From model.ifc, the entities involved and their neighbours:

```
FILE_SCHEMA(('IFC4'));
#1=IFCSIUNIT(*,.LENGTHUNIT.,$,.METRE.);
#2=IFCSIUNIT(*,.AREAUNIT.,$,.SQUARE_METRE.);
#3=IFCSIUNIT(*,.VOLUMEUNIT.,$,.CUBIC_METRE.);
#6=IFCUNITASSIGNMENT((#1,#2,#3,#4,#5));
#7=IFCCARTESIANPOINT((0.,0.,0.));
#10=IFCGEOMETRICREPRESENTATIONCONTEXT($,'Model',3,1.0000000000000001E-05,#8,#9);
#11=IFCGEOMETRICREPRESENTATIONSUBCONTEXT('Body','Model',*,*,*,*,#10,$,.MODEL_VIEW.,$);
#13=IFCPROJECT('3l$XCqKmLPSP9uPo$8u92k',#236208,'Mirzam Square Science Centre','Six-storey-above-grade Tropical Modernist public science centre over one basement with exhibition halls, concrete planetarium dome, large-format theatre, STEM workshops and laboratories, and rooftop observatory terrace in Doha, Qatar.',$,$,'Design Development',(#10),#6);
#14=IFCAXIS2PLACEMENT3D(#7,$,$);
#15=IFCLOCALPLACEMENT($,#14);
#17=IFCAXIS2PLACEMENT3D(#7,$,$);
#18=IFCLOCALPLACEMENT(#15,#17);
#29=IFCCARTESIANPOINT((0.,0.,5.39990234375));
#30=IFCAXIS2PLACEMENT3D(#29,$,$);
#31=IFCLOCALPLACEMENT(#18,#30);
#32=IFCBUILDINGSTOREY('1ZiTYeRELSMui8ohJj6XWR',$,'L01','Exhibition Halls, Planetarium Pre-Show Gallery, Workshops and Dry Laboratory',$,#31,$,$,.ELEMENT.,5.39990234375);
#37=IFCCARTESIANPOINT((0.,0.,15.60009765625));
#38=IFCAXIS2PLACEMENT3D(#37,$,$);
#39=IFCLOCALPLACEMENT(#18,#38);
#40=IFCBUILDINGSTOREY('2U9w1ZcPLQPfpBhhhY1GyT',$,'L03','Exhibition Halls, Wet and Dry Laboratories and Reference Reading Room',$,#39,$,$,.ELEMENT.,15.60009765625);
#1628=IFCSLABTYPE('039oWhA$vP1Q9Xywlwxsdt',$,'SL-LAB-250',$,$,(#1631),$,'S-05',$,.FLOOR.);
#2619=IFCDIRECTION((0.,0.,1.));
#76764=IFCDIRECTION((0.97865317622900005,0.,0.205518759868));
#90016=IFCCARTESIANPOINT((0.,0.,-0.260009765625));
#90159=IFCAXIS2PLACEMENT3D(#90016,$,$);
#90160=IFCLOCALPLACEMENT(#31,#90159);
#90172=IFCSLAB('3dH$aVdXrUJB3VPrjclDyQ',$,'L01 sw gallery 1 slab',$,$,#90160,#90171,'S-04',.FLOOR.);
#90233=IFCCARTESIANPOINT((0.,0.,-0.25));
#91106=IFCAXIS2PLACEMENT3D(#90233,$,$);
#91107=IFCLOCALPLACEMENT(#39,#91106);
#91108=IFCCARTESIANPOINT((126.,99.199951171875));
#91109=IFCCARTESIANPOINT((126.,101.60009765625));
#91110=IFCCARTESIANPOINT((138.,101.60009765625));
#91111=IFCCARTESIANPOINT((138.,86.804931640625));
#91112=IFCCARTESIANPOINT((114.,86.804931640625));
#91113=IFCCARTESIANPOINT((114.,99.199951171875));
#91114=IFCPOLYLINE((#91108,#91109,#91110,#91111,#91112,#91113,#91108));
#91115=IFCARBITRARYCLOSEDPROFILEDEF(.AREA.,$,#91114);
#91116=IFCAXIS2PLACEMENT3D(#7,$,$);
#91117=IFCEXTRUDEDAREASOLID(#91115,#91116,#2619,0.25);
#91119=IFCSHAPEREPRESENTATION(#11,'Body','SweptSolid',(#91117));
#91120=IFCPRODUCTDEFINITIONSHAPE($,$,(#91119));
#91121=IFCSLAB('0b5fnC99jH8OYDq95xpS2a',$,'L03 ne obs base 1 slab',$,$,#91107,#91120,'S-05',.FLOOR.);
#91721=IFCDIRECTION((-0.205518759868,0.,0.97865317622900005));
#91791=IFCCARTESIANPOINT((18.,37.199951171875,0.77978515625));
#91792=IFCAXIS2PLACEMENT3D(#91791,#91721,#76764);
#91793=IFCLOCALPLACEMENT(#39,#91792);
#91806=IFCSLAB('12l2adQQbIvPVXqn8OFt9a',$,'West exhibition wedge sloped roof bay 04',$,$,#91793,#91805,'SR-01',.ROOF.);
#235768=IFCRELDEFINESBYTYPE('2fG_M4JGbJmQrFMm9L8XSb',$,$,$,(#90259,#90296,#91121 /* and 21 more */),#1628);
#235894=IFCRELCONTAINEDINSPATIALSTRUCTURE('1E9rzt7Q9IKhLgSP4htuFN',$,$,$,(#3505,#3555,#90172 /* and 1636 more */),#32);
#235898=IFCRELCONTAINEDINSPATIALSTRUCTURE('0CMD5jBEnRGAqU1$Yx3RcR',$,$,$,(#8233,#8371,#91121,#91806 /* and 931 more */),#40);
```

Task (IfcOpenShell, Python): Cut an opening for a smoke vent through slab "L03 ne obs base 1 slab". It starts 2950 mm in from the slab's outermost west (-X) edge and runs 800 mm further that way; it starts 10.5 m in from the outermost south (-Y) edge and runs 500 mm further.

```python
import numpy as np
import ifcopenshell
import ifcopenshell.api.feature
import ifcopenshell.api.geometry
import ifcopenshell.api.root
import ifcopenshell.geom
import ifcopenshell.util.placement
import ifcopenshell.util.representation
import ifcopenshell.util.shape
import ifcopenshell.util.unit

model = ifcopenshell.open("model.ifc")
unit_scale = ifcopenshell.util.unit.calculate_unit_scale(model)
settings = ifcopenshell.geom.settings()


def volume(element):
    """Net volume in cubic metres, openings subtracted."""
    shape = ifcopenshell.geom.create_shape(settings, element)
    return ifcopenshell.util.shape.get_volume(shape.geometry)


slab = model.by_guid("0b5fnC99jH8OYDq95xpS2a")
before = volume(slab)

# Extent in the slab's own axes, in metres. The edges named are its -X and -Y sides.
slab_shape = ifcopenshell.geom.create_shape(settings, slab)
vertices = ifcopenshell.util.shape.get_vertices(slab_shape.geometry)
x_min, y_min, bottom = vertices.min(axis=0)
top = vertices[:, 2].max()

opening = ifcopenshell.api.root.create_entity(model, ifc_class="IfcOpeningElement", name="Smoke vent opening", predefined_type="OPENING")
context = ifcopenshell.util.representation.get_context(model, "Model", "Body", "MODEL_VIEW")
width, depth = 0.8, 0.5
outline = [(0.0, 0.0), (width, 0.0), (width, depth), (0.0, depth), (0.0, 0.0)]
# Overshoot both faces by 50 mm so the cut is clean.
shape = ifcopenshell.api.geometry.add_slab_representation(
    model, context=context, depth=top - bottom + 0.1, polyline=outline
)
ifcopenshell.api.geometry.assign_representation(model, product=opening, representation=shape)

matrix = ifcopenshell.util.placement.get_local_placement(slab.ObjectPlacement)
matrix[:, 3] = matrix @ np.append(np.array([x_min + 2.95, y_min + 10.5, bottom - 0.05]) / unit_scale, 1.0)
ifcopenshell.api.geometry.edit_object_placement(model, product=opening, matrix=matrix, is_si=False)
ifcopenshell.api.feature.add_feature(model, feature=opening, element=slab)

after = volume(slab)

print(f"slab volume {before:.3f} -> {after:.3f} m3")

model.write("model_rev.ifc")
```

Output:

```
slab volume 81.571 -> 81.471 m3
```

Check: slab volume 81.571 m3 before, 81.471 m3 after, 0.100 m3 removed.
